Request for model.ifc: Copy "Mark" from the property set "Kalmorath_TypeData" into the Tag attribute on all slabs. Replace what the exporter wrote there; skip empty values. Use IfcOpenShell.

First a look at what the model holds.

```python
import ifcopenshell
import ifcopenshell.util.element

model = ifcopenshell.open("model.ifc")
print(model.schema)
slabs = model.by_type("IfcSlab")
print(len(slabs), "slabs")
for e in slabs[:8]:
    source = ifcopenshell.util.element.get_pset(e, "Kalmorath_TypeData", "Mark")
    target = e.Tag
    print(e.id(), repr(source), repr(target), sep=" | ")
```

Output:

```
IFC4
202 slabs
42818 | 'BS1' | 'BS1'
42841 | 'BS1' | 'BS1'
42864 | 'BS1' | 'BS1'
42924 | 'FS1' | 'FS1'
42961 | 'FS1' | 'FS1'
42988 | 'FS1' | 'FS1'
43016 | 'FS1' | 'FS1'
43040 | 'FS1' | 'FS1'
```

```python
import ifcopenshell
import ifcopenshell.util.element

model = ifcopenshell.open("model.ifc")

count = 0
for e in model.by_type("IfcSlab"):
    value = ifcopenshell.util.element.get_pset(e, "Kalmorath_TypeData", "Mark")
    current = e.Tag
    if not value or not value.strip() or current == value:
        continue
    e.Tag = value
    count += 1

print(count, "slabs updated")

model.write("model_edited.ifc")
```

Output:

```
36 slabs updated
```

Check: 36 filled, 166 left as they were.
